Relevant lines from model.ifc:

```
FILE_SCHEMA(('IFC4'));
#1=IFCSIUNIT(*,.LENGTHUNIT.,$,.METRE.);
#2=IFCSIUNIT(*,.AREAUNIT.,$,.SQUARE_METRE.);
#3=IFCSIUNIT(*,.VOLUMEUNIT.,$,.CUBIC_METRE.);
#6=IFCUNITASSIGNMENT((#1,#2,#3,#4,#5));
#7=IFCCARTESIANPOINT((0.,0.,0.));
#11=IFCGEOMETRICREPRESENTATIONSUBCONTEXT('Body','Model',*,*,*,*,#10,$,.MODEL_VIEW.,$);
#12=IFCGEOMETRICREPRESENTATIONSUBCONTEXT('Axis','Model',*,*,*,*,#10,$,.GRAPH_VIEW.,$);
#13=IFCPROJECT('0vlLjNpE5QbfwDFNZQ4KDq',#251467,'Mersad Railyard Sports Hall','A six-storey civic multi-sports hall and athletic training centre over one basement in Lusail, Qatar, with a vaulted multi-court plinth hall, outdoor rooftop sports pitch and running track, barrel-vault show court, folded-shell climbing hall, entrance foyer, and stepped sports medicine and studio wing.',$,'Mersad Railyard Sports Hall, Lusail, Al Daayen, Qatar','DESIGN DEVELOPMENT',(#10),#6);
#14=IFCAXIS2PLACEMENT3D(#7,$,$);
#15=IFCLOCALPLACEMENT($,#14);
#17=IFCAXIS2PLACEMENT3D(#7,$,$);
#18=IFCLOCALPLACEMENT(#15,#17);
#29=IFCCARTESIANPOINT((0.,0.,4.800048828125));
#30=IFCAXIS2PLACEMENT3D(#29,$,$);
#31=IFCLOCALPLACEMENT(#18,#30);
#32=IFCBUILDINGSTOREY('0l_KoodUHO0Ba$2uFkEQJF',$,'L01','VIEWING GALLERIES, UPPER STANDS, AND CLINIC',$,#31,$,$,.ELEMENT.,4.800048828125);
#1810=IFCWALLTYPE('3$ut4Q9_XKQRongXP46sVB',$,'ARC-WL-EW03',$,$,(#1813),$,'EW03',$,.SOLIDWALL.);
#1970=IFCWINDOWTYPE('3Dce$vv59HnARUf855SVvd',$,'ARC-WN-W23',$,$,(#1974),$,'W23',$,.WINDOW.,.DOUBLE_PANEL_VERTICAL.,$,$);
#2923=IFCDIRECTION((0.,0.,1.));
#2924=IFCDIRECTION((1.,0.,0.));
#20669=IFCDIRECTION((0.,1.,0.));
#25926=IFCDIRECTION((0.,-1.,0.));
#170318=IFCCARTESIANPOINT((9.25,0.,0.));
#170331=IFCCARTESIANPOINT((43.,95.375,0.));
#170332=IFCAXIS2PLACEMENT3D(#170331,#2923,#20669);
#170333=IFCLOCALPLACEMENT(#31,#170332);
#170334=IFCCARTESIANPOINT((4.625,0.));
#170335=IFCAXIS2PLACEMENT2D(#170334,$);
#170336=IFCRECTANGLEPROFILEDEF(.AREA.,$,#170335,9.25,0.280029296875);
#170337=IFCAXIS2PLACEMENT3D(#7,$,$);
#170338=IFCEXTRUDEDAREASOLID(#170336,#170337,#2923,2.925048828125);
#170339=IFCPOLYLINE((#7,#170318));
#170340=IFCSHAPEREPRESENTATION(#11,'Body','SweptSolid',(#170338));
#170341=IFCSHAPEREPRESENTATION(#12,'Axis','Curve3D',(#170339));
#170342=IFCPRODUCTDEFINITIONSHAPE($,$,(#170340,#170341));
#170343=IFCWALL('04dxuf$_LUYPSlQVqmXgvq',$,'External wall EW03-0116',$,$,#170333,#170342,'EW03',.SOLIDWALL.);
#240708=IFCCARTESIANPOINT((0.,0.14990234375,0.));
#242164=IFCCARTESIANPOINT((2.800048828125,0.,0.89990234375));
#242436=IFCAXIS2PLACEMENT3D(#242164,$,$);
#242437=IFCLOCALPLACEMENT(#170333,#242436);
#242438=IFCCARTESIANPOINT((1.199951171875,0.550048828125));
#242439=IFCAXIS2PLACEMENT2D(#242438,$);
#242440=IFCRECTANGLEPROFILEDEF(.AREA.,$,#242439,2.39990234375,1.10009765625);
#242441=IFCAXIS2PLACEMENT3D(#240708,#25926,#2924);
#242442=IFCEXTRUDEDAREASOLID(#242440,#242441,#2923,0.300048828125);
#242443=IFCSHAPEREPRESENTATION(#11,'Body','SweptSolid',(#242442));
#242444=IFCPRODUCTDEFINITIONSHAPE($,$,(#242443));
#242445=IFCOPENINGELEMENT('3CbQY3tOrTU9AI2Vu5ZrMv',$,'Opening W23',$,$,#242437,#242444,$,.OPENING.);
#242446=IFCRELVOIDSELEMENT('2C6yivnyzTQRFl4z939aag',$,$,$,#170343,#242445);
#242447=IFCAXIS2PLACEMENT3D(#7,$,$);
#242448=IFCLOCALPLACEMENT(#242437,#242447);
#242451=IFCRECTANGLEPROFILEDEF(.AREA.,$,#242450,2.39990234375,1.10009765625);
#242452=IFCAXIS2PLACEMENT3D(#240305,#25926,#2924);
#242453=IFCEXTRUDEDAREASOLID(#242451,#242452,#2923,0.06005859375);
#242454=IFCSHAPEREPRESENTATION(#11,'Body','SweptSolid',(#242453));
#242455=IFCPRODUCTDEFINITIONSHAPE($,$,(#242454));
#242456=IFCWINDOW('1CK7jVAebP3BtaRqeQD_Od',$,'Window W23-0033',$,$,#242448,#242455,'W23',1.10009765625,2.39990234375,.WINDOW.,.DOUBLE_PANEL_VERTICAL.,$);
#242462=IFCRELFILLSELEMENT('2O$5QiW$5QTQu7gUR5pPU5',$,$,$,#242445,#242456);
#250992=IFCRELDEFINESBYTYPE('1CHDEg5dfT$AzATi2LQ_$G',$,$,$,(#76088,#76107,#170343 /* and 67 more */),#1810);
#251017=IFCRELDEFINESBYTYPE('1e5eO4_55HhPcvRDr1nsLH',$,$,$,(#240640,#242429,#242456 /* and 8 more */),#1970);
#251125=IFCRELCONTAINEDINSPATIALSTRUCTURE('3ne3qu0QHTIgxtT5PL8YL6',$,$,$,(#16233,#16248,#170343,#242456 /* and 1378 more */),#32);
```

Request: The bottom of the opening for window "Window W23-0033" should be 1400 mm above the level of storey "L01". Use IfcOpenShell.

```python
import numpy as np
import ifcopenshell
import ifcopenshell.api.geometry
import ifcopenshell.geom
import ifcopenshell.util.element
import ifcopenshell.util.placement
import ifcopenshell.util.shape
import ifcopenshell.util.unit

model = ifcopenshell.open("model.ifc")
unit_scale = ifcopenshell.util.unit.calculate_unit_scale(model)

window = model.by_guid("1CK7jVAebP3BtaRqeQD_Od")
opening = window.FillsVoids[0].RelatingOpeningElement
storey = ifcopenshell.util.element.get_container(window, ifc_class="IfcBuildingStorey")
level = ifcopenshell.util.placement.get_local_placement(storey.ObjectPlacement)[2, 3]

# The opening's origin need not be at the sill, so measure its lowest point.
shape = ifcopenshell.geom.create_shape(ifcopenshell.geom.settings(), opening)
bottom = ifcopenshell.util.shape.get_shape_bottom_elevation(shape, shape.geometry) / unit_scale
dz = level + 1.4 / unit_scale - bottom

shift = np.array([0.0, 0.0, dz])
# The window is placed relative to its opening, so it follows when the opening moves.
matrix = ifcopenshell.util.placement.get_local_placement(opening.ObjectPlacement)
matrix[:3, 3] += shift
ifcopenshell.api.geometry.edit_object_placement(
    model, product=opening, matrix=matrix, is_si=False, should_transform_children=True
)

print(f"moved by {dz * unit_scale:+.3f} m")

model.write("model_v2.ifc")
```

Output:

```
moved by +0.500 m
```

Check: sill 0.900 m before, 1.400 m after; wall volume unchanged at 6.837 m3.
